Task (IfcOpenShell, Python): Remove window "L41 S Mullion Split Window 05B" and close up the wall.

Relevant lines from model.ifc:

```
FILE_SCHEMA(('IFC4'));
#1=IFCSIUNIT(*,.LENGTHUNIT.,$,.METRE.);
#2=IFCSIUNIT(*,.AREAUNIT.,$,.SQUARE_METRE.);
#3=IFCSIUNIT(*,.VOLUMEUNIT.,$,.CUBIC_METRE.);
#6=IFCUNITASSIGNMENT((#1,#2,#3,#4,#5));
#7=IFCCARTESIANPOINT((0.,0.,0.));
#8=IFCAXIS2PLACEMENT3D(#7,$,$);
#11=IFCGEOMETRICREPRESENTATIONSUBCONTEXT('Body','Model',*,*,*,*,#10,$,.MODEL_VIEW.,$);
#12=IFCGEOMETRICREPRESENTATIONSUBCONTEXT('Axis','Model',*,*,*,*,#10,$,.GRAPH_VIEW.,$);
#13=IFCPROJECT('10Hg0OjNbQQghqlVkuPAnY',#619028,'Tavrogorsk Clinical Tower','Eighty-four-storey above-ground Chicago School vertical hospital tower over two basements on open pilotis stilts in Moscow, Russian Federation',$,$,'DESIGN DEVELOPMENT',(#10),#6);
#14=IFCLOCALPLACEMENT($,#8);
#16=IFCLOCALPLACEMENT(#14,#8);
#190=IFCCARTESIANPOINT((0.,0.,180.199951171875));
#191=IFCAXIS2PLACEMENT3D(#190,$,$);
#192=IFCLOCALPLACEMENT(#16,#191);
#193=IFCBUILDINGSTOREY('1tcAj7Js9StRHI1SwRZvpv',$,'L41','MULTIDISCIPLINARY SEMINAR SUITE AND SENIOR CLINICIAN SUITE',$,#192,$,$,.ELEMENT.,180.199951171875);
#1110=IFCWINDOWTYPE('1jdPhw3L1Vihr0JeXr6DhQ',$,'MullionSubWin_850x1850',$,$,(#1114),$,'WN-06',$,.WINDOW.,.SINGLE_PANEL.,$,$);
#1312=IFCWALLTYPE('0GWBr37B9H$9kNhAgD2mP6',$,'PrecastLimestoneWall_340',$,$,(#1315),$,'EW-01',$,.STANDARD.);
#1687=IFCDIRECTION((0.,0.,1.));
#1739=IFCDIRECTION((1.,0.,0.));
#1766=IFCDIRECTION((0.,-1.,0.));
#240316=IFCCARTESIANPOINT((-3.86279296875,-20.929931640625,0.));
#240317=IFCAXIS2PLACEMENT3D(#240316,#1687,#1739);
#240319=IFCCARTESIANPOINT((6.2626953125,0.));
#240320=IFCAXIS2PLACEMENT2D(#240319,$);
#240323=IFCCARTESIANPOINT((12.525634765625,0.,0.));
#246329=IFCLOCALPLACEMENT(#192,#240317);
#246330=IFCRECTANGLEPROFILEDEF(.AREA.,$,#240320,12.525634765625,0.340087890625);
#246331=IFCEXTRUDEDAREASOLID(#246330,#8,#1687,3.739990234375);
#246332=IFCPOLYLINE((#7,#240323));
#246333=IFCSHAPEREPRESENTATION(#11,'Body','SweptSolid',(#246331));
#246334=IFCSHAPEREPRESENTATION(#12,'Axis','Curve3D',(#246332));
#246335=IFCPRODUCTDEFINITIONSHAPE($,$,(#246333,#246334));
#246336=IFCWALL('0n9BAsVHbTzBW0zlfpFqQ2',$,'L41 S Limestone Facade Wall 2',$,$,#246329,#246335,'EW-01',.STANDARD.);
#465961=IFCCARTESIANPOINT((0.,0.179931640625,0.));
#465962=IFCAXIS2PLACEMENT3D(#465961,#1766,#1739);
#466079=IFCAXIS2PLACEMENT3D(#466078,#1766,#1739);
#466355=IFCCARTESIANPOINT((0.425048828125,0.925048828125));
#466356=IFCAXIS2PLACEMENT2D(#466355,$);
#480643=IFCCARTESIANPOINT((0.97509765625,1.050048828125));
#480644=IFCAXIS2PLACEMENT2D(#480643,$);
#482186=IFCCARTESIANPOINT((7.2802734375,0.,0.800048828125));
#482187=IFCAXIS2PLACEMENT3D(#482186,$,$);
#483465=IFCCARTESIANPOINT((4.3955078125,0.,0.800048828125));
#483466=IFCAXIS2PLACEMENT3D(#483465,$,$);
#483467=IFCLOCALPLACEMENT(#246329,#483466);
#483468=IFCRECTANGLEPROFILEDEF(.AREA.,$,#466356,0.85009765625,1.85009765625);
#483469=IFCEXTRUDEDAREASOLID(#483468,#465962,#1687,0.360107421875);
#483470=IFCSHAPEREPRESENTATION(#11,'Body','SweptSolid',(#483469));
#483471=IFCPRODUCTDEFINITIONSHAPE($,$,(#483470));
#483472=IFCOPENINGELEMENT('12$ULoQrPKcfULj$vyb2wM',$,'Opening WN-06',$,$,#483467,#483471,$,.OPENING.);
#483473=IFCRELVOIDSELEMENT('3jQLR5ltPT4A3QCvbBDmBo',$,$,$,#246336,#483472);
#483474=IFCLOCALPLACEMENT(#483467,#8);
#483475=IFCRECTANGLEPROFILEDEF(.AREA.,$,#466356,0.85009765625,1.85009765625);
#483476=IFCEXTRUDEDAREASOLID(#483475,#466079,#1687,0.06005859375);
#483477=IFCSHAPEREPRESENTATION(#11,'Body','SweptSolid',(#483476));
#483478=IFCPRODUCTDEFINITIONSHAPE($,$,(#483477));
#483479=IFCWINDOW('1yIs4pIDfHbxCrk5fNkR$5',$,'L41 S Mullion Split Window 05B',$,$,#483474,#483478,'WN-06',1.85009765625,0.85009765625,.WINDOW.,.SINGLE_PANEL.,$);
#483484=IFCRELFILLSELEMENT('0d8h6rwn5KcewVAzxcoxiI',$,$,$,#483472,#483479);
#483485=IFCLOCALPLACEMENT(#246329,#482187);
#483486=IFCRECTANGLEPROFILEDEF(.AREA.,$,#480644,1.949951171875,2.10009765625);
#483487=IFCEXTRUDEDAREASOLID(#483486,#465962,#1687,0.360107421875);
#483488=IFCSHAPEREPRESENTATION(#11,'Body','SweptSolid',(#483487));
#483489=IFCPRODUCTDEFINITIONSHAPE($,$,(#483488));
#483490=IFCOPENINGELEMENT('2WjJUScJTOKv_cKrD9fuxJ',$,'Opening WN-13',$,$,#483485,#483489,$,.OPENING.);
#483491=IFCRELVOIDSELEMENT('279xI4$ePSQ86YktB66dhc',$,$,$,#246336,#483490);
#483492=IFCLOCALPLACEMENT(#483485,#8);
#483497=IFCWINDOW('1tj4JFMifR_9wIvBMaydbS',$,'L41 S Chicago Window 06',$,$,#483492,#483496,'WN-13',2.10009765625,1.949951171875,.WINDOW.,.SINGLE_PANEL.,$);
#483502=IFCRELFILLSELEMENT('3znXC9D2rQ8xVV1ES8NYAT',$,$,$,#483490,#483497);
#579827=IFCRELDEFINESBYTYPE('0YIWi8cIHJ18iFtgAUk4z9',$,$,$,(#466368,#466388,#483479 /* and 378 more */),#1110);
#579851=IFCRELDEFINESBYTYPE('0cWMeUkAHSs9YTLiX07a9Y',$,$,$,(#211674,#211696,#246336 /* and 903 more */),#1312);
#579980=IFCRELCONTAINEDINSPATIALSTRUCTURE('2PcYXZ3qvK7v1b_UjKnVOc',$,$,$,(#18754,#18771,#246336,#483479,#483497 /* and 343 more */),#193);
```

```python
import ifcopenshell
import ifcopenshell.api.feature
import ifcopenshell.api.root
import ifcopenshell.geom
import ifcopenshell.util.shape

model = ifcopenshell.open("model.ifc")
settings = ifcopenshell.geom.settings()


def volume(element):
    """Net volume in cubic metres, openings subtracted."""
    shape = ifcopenshell.geom.create_shape(settings, element)
    return ifcopenshell.util.shape.get_volume(shape.geometry)


window = model.by_id(483479)
opening = window.FillsVoids[0].RelatingOpeningElement
wall = opening.VoidsElements[0].RelatingBuildingElement
before = volume(wall)

ifcopenshell.api.root.remove_product(model, product=window)
ifcopenshell.api.feature.remove_feature(model, feature=opening)

after = volume(wall)

print(f"wall volume {before:.3f} -> {after:.3f} m3")

model.write("model_v2.ifc")
```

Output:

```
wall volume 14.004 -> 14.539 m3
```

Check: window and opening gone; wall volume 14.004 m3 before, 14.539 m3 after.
